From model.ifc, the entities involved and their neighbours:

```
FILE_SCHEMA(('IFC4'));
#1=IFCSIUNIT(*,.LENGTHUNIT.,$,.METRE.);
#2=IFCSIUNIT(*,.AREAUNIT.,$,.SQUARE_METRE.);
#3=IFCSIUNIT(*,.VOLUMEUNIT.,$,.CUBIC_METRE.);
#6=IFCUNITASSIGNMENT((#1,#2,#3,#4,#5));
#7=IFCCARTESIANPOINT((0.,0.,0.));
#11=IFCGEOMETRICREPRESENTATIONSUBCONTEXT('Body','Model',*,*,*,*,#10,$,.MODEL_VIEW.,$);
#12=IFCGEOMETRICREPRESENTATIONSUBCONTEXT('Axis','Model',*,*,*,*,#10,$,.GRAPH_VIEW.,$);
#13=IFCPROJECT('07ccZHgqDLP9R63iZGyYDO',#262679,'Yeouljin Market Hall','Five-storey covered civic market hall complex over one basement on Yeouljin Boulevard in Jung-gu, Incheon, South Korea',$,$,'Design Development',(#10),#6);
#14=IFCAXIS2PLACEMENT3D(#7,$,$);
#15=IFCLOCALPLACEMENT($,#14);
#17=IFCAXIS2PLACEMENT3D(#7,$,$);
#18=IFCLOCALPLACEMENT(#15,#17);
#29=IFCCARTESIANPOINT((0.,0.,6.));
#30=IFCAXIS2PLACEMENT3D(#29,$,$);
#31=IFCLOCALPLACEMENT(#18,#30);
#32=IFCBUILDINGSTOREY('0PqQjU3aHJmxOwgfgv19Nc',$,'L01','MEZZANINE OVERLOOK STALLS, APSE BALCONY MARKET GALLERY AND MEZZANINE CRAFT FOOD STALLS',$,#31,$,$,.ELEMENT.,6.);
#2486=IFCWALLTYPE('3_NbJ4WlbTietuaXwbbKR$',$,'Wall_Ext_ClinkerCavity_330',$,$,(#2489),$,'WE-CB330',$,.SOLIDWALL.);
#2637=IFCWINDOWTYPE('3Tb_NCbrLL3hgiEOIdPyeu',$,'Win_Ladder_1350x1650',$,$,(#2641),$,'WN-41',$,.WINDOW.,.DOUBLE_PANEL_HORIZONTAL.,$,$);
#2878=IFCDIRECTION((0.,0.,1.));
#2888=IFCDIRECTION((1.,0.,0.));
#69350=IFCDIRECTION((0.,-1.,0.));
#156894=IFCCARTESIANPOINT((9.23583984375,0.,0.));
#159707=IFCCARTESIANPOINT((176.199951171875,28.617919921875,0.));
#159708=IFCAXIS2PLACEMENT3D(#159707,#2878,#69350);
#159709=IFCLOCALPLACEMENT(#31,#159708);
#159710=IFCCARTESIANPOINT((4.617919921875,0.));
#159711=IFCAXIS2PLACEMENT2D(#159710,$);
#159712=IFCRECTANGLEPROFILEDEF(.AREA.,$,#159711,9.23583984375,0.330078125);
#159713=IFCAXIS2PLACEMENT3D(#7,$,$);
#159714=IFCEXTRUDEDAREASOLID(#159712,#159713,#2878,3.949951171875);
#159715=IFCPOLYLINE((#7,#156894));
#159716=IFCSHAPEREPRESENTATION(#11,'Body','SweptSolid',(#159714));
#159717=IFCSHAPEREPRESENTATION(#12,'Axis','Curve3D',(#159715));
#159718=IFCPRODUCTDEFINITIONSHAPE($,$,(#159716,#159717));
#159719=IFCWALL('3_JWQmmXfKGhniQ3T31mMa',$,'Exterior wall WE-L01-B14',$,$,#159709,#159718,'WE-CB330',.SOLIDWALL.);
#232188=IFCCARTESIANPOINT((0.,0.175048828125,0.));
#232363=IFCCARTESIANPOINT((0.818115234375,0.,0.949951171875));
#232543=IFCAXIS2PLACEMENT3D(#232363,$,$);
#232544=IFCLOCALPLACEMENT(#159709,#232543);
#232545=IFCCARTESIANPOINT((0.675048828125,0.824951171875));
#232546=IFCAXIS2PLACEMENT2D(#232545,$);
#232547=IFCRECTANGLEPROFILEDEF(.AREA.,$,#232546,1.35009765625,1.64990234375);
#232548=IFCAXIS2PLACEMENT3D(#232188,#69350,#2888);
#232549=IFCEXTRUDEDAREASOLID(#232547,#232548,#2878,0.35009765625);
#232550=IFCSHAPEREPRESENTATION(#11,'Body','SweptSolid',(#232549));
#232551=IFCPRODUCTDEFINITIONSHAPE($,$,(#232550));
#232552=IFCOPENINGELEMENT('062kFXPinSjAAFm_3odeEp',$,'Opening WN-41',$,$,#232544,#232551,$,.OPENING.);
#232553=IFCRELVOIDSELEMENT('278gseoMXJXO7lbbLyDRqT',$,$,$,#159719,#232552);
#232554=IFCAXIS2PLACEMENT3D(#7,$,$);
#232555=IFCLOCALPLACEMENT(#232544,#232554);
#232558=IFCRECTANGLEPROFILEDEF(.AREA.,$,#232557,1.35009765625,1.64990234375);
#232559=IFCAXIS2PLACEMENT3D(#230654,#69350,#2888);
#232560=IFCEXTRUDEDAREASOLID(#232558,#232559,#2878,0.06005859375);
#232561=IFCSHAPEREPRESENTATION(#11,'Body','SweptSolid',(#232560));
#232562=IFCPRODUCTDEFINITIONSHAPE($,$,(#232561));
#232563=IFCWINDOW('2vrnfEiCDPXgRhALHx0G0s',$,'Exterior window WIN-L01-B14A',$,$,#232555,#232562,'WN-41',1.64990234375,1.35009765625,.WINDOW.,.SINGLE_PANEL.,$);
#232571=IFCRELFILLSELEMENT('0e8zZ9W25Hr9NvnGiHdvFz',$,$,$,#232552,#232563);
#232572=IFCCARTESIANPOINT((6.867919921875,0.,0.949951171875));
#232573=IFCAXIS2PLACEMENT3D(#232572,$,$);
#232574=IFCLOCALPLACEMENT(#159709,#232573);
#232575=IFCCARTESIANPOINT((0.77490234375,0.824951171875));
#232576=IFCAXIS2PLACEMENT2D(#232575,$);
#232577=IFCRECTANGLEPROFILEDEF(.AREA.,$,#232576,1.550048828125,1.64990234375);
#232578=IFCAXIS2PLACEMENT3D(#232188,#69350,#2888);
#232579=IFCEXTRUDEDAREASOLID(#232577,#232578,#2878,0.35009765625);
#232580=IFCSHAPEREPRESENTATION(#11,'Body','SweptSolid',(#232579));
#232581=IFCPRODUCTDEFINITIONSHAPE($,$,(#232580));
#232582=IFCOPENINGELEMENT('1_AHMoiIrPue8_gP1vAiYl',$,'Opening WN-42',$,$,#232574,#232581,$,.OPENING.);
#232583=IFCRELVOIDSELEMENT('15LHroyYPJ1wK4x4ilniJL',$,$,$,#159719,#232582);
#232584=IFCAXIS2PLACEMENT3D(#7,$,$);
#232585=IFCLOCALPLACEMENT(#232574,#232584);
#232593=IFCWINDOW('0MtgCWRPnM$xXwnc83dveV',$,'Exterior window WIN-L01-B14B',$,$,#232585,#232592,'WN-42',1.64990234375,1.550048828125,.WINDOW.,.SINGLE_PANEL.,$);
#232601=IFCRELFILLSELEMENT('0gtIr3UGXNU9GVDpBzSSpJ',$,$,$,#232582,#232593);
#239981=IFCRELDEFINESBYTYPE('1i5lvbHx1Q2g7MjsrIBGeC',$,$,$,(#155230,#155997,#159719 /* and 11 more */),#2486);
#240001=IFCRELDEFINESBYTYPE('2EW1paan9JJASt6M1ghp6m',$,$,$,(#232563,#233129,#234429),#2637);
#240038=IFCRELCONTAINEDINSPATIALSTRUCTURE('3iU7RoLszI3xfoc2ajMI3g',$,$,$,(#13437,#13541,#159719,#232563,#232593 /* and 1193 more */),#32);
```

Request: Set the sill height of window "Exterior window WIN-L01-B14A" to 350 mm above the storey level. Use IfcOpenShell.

```python
import numpy as np
import ifcopenshell
import ifcopenshell.api.geometry
import ifcopenshell.geom
import ifcopenshell.util.element
import ifcopenshell.util.placement
import ifcopenshell.util.shape
import ifcopenshell.util.unit

model = ifcopenshell.open("model.ifc")
unit_scale = ifcopenshell.util.unit.calculate_unit_scale(model)

window = model.by_guid("2vrnfEiCDPXgRhALHx0G0s")
opening = window.FillsVoids[0].RelatingOpeningElement
storey = ifcopenshell.util.element.get_container(window, ifc_class="IfcBuildingStorey")
level = ifcopenshell.util.placement.get_local_placement(storey.ObjectPlacement)[2, 3]

# The opening's origin need not be at the sill, so measure its lowest point.
shape = ifcopenshell.geom.create_shape(ifcopenshell.geom.settings(), opening)
bottom = ifcopenshell.util.shape.get_shape_bottom_elevation(shape, shape.geometry) / unit_scale
dz = level + 0.35 / unit_scale - bottom

shift = np.array([0.0, 0.0, dz])
# The window is placed relative to its opening, so it follows when the opening moves.
matrix = ifcopenshell.util.placement.get_local_placement(opening.ObjectPlacement)
matrix[:3, 3] += shift
ifcopenshell.api.geometry.edit_object_placement(
    model, product=opening, matrix=matrix, is_si=False, should_transform_children=True
)

print(f"moved by {dz * unit_scale:+.3f} m")

model.write("model_edited.ifc")
```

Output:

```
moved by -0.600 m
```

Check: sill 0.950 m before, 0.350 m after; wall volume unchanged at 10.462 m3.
